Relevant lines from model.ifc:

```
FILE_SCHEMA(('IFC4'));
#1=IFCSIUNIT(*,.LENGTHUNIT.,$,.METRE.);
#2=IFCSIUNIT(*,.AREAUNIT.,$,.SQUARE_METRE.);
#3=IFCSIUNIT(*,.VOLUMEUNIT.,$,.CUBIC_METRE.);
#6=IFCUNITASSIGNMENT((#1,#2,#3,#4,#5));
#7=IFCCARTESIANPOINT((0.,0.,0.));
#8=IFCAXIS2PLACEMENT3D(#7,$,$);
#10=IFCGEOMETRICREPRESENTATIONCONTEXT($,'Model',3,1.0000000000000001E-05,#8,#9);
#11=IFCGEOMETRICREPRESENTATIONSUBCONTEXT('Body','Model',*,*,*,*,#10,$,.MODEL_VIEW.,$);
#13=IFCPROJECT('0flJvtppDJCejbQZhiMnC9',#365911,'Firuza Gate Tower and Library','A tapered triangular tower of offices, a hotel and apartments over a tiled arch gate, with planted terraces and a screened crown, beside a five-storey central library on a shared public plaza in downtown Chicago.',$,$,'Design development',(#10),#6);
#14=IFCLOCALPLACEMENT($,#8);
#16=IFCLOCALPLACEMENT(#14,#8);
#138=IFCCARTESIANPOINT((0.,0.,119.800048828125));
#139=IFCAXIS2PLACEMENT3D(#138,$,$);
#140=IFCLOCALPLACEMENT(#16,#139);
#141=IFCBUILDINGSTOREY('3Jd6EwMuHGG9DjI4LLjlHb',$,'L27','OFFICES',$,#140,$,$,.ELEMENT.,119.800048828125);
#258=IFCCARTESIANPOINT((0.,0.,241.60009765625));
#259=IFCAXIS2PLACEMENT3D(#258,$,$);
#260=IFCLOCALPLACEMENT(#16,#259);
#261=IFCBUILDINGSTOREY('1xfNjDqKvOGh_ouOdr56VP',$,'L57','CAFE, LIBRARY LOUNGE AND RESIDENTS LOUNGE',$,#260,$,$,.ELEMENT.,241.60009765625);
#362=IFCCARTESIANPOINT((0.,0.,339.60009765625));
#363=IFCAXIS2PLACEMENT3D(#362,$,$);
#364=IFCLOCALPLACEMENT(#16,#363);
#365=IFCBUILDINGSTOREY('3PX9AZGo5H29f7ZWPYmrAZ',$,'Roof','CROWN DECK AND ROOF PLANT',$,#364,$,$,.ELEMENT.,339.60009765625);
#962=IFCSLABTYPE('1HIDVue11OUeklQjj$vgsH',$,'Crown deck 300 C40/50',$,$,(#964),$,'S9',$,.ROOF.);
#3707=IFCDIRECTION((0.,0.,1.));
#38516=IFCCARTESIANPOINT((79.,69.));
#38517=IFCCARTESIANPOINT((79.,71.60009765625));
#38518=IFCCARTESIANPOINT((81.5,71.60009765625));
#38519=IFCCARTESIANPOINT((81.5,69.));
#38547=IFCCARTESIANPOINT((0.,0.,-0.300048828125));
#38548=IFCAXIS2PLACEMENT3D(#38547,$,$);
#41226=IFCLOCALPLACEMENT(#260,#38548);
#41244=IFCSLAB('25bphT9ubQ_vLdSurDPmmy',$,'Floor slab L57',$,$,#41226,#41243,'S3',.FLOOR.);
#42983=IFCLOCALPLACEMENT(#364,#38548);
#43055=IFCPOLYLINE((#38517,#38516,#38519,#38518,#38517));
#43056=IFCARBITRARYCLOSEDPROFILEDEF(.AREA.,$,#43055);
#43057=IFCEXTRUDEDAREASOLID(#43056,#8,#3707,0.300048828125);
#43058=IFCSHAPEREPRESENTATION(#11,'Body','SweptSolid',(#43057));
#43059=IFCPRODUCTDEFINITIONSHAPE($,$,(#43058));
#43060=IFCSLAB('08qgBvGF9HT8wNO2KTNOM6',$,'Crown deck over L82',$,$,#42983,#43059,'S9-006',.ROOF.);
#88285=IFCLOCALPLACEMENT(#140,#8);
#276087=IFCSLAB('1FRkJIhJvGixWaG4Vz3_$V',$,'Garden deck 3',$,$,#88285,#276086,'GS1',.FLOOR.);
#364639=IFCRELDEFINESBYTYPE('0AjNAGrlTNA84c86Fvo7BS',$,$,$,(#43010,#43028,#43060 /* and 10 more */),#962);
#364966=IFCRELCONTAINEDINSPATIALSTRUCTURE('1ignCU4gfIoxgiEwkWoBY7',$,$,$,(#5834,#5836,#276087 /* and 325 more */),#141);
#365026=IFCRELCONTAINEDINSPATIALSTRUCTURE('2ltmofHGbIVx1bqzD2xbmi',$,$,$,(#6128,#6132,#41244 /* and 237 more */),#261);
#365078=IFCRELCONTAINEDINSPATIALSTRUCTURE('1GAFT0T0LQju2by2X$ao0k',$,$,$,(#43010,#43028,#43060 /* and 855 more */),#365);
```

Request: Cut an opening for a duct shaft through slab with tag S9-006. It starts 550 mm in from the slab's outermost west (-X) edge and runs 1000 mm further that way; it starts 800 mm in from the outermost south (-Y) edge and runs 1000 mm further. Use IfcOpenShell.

```python
import numpy as np
import ifcopenshell
import ifcopenshell.api.feature
import ifcopenshell.api.geometry
import ifcopenshell.api.root
import ifcopenshell.geom
import ifcopenshell.util.placement
import ifcopenshell.util.representation
import ifcopenshell.util.shape
import ifcopenshell.util.unit

model = ifcopenshell.open("model.ifc")
unit_scale = ifcopenshell.util.unit.calculate_unit_scale(model)
settings = ifcopenshell.geom.settings()


def volume(element):
    """Net volume in cubic metres, openings subtracted."""
    shape = ifcopenshell.geom.create_shape(settings, element)
    return ifcopenshell.util.shape.get_volume(shape.geometry)


slab = model.by_guid("08qgBvGF9HT8wNO2KTNOM6")
before = volume(slab)

# Extent in the slab's own axes, in metres. The edges named are its -X and -Y sides.
slab_shape = ifcopenshell.geom.create_shape(settings, slab)
vertices = ifcopenshell.util.shape.get_vertices(slab_shape.geometry)
x_min, y_min, bottom = vertices.min(axis=0)
top = vertices[:, 2].max()

opening = ifcopenshell.api.root.create_entity(model, ifc_class="IfcOpeningElement", name="Duct shaft opening", predefined_type="OPENING")
context = ifcopenshell.util.representation.get_context(model, "Model", "Body", "MODEL_VIEW")
width, depth = 1, 1
outline = [(0.0, 0.0), (width, 0.0), (width, depth), (0.0, depth), (0.0, 0.0)]
# Overshoot both faces by 50 mm so the cut is clean.
shape = ifcopenshell.api.geometry.add_slab_representation(
    model, context=context, depth=top - bottom + 0.1, polyline=outline
)
ifcopenshell.api.geometry.assign_representation(model, product=opening, representation=shape)

matrix = ifcopenshell.util.placement.get_local_placement(slab.ObjectPlacement)
matrix[:, 3] = matrix @ np.append(np.array([x_min + 0.55, y_min + 0.8, bottom - 0.05]) / unit_scale, 1.0)
ifcopenshell.api.geometry.edit_object_placement(model, product=opening, matrix=matrix, is_si=False)
ifcopenshell.api.feature.add_feature(model, feature=opening, element=slab)

after = volume(slab)

print(f"slab volume {before:.3f} -> {after:.3f} m3")

model.write("model_v2.ifc")
```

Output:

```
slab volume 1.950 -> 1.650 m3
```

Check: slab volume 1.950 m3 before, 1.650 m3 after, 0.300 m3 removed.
